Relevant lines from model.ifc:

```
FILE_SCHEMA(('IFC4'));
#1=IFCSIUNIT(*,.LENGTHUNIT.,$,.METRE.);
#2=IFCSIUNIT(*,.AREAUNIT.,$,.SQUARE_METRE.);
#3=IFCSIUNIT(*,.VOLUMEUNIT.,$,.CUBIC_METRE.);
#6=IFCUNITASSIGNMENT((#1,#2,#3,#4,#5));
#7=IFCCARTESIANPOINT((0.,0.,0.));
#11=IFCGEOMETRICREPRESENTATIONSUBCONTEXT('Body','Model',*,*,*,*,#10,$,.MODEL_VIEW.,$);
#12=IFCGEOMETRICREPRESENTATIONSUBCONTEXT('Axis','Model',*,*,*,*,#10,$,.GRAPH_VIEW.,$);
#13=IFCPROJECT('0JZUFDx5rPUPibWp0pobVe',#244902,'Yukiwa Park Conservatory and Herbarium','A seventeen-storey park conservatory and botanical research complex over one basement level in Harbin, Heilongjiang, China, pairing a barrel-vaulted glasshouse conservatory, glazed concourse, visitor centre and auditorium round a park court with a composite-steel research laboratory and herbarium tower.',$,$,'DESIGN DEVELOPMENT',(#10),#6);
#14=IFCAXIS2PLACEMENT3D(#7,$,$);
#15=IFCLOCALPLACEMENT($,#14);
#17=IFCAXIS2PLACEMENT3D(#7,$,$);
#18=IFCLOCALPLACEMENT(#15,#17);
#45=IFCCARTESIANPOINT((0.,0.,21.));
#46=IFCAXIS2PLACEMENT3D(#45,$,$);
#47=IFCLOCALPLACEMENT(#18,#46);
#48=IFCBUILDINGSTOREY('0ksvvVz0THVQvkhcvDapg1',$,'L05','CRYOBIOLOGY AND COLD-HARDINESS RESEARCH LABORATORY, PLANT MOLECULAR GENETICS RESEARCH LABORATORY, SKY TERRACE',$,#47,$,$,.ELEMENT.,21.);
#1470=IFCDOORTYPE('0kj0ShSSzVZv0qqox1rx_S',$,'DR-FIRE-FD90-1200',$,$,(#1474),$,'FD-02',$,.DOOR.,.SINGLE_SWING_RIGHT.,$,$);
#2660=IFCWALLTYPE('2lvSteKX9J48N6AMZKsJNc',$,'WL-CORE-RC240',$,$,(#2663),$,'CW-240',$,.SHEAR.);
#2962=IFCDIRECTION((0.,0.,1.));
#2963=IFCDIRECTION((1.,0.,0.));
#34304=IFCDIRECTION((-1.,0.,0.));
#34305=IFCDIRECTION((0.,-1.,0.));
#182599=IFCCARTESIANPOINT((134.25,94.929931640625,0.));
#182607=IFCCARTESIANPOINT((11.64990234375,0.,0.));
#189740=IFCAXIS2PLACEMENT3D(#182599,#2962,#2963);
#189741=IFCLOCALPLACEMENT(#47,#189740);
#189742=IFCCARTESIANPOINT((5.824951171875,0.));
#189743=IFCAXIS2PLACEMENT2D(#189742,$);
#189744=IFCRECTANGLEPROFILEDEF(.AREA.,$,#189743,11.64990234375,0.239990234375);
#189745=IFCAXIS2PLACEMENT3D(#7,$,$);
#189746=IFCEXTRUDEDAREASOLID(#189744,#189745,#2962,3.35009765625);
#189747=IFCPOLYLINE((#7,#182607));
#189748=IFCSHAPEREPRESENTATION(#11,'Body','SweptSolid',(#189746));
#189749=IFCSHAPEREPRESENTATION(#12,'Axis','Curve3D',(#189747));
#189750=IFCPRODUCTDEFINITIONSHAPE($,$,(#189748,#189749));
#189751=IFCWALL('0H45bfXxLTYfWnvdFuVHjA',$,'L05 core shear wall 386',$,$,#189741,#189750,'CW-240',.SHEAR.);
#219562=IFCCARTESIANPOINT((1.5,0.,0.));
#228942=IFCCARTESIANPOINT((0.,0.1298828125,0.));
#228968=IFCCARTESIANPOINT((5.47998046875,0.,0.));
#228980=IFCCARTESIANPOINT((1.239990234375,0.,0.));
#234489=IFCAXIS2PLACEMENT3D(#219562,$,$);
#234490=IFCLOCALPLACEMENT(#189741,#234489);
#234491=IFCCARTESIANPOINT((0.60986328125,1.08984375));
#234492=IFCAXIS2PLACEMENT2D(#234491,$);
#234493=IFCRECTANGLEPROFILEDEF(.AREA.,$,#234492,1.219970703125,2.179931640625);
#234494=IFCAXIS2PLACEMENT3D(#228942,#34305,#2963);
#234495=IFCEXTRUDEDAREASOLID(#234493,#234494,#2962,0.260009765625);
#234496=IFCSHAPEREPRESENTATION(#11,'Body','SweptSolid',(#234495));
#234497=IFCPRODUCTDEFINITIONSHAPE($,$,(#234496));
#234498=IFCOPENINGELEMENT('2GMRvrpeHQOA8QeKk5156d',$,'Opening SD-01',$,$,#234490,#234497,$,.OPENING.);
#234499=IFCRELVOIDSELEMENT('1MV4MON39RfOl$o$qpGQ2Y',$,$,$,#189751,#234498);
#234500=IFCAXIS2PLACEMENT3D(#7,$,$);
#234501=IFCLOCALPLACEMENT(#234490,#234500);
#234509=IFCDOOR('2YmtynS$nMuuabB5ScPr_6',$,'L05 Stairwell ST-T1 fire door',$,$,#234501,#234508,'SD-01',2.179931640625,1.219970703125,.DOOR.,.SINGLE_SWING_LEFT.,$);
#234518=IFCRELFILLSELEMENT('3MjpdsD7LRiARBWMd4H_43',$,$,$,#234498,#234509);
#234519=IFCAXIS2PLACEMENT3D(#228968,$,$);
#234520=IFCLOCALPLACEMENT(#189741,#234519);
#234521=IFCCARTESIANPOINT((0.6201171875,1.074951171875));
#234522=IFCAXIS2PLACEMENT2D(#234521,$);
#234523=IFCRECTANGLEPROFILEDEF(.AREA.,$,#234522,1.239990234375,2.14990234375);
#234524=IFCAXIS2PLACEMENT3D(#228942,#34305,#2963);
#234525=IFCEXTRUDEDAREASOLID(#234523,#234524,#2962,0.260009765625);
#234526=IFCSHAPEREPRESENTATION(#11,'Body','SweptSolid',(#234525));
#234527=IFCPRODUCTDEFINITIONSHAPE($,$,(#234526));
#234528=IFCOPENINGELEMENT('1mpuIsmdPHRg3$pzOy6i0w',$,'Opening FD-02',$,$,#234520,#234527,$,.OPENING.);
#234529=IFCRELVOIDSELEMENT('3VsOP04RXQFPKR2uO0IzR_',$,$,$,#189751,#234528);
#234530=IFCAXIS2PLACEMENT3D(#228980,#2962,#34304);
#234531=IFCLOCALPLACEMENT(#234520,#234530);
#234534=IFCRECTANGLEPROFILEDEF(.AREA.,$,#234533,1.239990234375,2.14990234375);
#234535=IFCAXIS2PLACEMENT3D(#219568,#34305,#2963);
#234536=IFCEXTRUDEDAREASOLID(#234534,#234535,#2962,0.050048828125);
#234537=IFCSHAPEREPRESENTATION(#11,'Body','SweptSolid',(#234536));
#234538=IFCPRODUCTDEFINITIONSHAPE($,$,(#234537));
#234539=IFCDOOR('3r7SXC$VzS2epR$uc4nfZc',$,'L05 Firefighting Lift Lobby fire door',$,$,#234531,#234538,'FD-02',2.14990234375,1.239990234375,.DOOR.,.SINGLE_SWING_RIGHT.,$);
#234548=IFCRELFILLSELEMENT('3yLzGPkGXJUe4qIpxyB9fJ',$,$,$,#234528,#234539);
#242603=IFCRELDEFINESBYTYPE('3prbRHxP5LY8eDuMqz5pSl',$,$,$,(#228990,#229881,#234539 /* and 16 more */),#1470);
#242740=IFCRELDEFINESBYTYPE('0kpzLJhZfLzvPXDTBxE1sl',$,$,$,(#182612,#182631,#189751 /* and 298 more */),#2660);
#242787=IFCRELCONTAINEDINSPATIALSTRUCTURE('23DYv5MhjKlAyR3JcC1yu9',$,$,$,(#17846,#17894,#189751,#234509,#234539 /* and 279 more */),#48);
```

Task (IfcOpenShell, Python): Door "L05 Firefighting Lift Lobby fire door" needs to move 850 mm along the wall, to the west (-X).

```python
import ifcopenshell
import ifcopenshell.api.geometry
import ifcopenshell.util.placement
import ifcopenshell.util.unit

model = ifcopenshell.open("model.ifc")
unit_scale = ifcopenshell.util.unit.calculate_unit_scale(model)

door = model.by_guid("3r7SXC$VzS2epR$uc4nfZc")
opening = door.FillsVoids[0].RelatingOpeningElement
wall = opening.VoidsElements[0].RelatingBuildingElement

wall_matrix = ifcopenshell.util.placement.get_local_placement(wall.ObjectPlacement)
shift = wall_matrix[:3, 0] * -0.85 / unit_scale
before = ifcopenshell.util.placement.get_local_placement(door.ObjectPlacement)[:3, 3].copy()

# The door is placed relative to its opening, so it follows when the opening moves.
matrix = ifcopenshell.util.placement.get_local_placement(opening.ObjectPlacement)
matrix[:3, 3] += shift
ifcopenshell.api.geometry.edit_object_placement(
    model, product=opening, matrix=matrix, is_si=False, should_transform_children=True
)

after = ifcopenshell.util.placement.get_local_placement(door.ObjectPlacement)[:3, 3]
print("door moved by", (after - before).round(3) + 0.0)

model.write("model_v2.ifc")
```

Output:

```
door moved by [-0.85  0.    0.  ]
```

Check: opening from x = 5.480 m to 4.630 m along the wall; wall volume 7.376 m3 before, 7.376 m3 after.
